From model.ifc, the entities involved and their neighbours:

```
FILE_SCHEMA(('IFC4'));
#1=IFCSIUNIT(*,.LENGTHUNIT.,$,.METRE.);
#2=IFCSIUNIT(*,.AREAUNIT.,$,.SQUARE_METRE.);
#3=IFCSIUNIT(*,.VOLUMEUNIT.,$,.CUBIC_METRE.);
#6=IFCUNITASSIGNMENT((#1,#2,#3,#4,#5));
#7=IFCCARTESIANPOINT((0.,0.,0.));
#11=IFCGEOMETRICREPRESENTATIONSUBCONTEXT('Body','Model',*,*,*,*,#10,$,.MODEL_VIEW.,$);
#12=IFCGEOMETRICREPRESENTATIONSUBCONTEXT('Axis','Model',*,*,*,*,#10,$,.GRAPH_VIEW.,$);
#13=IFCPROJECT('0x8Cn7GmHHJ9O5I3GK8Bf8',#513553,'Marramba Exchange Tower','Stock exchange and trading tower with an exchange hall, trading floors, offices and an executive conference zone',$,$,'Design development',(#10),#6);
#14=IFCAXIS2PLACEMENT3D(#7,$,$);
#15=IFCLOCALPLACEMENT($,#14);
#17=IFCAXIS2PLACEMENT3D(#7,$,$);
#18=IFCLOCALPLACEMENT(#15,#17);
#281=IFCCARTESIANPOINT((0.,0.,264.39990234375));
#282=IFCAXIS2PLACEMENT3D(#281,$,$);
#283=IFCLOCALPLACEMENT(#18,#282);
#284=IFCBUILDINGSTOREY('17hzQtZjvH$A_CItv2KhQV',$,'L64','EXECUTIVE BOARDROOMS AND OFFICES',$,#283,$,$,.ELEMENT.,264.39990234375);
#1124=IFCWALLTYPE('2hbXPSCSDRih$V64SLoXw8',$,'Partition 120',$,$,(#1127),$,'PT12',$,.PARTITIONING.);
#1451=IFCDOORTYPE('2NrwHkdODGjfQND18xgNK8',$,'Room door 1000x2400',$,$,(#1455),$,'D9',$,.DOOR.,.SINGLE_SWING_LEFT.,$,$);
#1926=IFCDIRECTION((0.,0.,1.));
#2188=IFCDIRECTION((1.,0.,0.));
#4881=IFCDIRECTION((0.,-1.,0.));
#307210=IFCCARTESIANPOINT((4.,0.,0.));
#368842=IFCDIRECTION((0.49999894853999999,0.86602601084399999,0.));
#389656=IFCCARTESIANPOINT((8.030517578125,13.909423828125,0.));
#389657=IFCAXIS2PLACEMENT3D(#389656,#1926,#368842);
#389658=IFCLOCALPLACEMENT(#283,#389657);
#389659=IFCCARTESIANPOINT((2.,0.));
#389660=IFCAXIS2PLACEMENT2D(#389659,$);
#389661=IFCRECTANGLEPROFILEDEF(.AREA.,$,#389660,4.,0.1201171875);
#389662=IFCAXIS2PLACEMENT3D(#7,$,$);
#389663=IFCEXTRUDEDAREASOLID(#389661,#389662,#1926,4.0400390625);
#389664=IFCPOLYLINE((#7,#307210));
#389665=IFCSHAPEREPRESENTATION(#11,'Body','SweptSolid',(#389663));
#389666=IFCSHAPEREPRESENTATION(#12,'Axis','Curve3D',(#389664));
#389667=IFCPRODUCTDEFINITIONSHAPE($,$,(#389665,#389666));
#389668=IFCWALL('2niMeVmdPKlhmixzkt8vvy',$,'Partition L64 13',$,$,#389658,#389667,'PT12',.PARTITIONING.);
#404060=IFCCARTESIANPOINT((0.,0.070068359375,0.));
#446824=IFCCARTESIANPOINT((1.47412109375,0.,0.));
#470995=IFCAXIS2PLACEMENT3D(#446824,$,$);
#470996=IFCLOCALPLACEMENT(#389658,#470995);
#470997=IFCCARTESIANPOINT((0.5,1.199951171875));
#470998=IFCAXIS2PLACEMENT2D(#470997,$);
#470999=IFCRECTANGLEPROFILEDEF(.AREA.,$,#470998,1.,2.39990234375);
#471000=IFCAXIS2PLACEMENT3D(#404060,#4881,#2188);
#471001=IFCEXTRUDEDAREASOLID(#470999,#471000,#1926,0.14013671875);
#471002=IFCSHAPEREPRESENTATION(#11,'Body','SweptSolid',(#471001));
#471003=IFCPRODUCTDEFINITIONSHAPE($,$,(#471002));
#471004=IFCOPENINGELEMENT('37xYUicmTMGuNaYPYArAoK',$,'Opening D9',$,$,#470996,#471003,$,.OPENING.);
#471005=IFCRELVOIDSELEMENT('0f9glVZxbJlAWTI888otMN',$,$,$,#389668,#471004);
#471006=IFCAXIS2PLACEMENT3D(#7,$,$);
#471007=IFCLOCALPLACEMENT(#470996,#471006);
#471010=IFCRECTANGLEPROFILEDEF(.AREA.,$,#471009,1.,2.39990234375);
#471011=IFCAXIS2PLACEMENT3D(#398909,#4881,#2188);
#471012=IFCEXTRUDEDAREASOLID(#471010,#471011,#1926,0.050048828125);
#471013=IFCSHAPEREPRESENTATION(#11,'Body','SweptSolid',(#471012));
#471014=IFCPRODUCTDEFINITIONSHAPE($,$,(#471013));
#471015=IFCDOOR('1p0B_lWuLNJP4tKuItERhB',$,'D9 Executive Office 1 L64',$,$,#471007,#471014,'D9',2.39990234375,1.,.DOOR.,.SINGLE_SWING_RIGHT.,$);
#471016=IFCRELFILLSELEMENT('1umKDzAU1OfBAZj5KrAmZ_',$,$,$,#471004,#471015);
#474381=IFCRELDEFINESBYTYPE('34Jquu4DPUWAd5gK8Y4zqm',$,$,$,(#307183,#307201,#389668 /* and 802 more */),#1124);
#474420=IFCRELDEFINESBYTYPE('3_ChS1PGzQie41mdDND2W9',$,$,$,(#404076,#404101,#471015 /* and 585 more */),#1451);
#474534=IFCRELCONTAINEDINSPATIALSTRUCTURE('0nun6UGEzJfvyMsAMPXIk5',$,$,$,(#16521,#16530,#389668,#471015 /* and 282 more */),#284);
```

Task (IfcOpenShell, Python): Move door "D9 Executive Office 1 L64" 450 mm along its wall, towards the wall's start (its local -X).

```python
import ifcopenshell
import ifcopenshell.api.geometry
import ifcopenshell.util.placement
import ifcopenshell.util.unit

model = ifcopenshell.open("model.ifc")
unit_scale = ifcopenshell.util.unit.calculate_unit_scale(model)

door = model.by_guid("1p0B_lWuLNJP4tKuItERhB")
opening = door.FillsVoids[0].RelatingOpeningElement
wall = opening.VoidsElements[0].RelatingBuildingElement

wall_matrix = ifcopenshell.util.placement.get_local_placement(wall.ObjectPlacement)
shift = wall_matrix[:3, 0] * -0.45 / unit_scale
before = ifcopenshell.util.placement.get_local_placement(door.ObjectPlacement)[:3, 3].copy()

# The door is placed relative to its opening, so it follows when the opening moves.
matrix = ifcopenshell.util.placement.get_local_placement(opening.ObjectPlacement)
matrix[:3, 3] += shift
ifcopenshell.api.geometry.edit_object_placement(
    model, product=opening, matrix=matrix, is_si=False, should_transform_children=True
)

after = ifcopenshell.util.placement.get_local_placement(door.ObjectPlacement)[:3, 3]
print("door moved by", (after - before).round(3) + 0.0)

model.write("model_edited.ifc")
```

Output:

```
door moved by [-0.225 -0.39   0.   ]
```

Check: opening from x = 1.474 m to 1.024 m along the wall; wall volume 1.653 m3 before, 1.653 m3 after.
